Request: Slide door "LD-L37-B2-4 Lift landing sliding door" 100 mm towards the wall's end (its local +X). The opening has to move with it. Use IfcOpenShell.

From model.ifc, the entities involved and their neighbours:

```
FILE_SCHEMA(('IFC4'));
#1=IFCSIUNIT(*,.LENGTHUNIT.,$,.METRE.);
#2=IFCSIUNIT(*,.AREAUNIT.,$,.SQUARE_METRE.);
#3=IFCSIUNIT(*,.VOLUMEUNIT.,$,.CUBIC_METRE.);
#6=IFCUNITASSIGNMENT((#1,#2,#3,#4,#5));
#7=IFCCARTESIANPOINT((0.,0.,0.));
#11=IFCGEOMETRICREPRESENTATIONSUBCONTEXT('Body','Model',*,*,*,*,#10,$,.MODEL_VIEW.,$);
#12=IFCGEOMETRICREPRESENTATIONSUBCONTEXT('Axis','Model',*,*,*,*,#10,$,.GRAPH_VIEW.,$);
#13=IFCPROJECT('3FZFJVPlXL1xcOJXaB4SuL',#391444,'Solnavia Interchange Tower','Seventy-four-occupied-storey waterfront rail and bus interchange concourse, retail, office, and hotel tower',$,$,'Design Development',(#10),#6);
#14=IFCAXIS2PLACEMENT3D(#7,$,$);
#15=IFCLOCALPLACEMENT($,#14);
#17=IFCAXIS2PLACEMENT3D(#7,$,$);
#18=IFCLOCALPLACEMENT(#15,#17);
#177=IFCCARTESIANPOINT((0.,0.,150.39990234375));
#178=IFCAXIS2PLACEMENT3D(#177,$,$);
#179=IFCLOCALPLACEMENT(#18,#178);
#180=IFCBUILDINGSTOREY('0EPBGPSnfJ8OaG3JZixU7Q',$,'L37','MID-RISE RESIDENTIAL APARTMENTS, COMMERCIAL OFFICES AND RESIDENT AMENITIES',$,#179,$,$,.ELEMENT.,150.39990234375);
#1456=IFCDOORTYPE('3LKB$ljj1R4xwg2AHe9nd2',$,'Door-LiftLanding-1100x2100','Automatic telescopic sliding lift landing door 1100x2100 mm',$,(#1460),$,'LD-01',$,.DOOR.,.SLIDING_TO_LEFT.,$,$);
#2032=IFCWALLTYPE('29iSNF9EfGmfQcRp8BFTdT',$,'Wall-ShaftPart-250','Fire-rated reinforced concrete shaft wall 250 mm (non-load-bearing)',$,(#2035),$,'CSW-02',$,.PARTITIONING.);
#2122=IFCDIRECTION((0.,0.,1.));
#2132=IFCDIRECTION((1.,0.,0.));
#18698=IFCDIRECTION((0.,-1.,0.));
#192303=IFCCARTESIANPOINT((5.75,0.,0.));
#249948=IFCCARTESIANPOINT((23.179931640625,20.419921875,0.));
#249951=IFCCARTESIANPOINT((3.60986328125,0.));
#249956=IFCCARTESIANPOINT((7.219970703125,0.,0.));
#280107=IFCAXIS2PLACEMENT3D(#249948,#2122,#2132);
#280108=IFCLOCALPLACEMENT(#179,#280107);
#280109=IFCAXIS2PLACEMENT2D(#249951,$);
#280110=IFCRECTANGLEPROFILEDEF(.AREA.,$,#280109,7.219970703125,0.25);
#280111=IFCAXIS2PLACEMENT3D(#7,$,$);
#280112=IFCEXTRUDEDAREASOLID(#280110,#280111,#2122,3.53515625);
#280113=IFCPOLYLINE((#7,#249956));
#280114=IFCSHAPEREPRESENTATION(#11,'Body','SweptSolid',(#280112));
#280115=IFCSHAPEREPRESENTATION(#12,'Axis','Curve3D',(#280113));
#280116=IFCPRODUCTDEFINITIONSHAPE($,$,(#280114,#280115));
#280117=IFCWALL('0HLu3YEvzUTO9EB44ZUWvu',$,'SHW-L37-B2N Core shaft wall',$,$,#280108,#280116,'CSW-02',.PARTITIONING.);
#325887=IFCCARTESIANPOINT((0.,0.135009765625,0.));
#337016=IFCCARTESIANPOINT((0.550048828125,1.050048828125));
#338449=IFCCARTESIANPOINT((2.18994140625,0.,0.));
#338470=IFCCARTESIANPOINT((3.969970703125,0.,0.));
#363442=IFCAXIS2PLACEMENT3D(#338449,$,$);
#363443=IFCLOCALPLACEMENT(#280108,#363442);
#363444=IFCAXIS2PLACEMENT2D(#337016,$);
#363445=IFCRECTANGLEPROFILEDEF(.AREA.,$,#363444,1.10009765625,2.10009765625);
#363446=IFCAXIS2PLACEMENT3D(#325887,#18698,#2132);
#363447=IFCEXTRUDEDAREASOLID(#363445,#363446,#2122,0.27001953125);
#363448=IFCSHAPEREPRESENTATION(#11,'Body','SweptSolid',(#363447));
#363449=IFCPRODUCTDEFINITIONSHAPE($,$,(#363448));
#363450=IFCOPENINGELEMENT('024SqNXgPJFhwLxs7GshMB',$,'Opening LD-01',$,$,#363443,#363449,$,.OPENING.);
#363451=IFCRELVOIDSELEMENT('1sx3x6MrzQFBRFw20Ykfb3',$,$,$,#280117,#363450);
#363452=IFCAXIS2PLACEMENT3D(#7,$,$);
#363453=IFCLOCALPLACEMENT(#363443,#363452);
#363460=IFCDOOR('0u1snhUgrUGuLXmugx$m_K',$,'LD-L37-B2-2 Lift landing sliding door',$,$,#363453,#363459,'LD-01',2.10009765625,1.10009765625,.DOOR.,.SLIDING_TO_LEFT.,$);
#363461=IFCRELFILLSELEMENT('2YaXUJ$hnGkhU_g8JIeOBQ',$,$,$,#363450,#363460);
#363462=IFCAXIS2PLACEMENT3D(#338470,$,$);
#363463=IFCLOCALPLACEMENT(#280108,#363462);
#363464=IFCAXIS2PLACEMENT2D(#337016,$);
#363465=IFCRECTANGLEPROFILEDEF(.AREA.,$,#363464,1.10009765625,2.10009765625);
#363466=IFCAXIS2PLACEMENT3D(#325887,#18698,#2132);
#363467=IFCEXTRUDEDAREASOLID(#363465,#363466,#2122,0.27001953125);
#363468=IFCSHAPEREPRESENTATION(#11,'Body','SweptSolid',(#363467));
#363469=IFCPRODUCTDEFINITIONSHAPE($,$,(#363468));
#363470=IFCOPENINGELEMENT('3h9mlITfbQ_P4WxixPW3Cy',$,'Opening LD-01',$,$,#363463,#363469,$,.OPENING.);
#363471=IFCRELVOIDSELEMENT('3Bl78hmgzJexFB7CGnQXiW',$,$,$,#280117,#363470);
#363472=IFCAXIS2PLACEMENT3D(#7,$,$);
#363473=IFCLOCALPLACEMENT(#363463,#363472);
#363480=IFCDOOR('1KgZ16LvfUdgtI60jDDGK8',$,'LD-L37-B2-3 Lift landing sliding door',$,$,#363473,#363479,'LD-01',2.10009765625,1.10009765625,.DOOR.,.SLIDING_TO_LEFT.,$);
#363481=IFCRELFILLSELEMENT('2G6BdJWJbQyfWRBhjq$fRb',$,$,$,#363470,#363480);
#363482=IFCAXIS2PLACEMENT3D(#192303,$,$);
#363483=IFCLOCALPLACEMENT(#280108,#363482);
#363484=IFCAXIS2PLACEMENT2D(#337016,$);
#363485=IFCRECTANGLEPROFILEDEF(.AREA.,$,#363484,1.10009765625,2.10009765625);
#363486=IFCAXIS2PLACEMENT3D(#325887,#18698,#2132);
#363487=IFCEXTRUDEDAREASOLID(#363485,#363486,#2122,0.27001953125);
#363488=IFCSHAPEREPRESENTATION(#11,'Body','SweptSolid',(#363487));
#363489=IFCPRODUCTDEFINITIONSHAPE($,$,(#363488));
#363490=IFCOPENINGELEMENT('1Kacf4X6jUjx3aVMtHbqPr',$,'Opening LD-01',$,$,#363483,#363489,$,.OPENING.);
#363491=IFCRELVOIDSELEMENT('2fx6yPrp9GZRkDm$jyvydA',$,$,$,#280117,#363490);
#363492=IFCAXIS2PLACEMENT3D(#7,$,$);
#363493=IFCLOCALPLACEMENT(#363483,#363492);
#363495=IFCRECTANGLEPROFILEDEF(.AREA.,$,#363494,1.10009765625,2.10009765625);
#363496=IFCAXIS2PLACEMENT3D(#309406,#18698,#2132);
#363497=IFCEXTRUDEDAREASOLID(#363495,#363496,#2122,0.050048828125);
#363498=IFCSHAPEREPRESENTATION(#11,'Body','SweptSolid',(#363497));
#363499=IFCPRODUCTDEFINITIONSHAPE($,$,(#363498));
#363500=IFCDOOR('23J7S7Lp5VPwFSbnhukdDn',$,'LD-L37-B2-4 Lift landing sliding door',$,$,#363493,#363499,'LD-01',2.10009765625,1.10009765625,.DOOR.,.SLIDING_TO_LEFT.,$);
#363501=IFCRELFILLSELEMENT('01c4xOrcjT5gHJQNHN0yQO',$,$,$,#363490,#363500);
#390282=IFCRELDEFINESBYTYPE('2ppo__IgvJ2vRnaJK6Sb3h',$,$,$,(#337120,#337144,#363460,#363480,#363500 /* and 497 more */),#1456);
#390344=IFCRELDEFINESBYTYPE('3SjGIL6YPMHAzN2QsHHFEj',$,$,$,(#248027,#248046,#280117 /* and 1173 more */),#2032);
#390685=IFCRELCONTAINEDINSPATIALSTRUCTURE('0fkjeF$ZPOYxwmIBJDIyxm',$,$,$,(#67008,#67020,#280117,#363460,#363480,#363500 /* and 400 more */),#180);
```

```python
import ifcopenshell
import ifcopenshell.api.geometry
import ifcopenshell.util.placement
import ifcopenshell.util.unit

model = ifcopenshell.open("model.ifc")
unit_scale = ifcopenshell.util.unit.calculate_unit_scale(model)

door = model.by_guid("23J7S7Lp5VPwFSbnhukdDn")
opening = door.FillsVoids[0].RelatingOpeningElement
wall = opening.VoidsElements[0].RelatingBuildingElement

wall_matrix = ifcopenshell.util.placement.get_local_placement(wall.ObjectPlacement)
shift = wall_matrix[:3, 0] * 0.1 / unit_scale
before = ifcopenshell.util.placement.get_local_placement(door.ObjectPlacement)[:3, 3].copy()

# The door is placed relative to its opening, so it follows when the opening moves.
matrix = ifcopenshell.util.placement.get_local_placement(opening.ObjectPlacement)
matrix[:3, 3] += shift
ifcopenshell.api.geometry.edit_object_placement(
    model, product=opening, matrix=matrix, is_si=False, should_transform_children=True
)

after = ifcopenshell.util.placement.get_local_placement(door.ObjectPlacement)[:3, 3]
print("door moved by", (after - before).round(3) + 0.0)

model.write("model_updated.ifc")
```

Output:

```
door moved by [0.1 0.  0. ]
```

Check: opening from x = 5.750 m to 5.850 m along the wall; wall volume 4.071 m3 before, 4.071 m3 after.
